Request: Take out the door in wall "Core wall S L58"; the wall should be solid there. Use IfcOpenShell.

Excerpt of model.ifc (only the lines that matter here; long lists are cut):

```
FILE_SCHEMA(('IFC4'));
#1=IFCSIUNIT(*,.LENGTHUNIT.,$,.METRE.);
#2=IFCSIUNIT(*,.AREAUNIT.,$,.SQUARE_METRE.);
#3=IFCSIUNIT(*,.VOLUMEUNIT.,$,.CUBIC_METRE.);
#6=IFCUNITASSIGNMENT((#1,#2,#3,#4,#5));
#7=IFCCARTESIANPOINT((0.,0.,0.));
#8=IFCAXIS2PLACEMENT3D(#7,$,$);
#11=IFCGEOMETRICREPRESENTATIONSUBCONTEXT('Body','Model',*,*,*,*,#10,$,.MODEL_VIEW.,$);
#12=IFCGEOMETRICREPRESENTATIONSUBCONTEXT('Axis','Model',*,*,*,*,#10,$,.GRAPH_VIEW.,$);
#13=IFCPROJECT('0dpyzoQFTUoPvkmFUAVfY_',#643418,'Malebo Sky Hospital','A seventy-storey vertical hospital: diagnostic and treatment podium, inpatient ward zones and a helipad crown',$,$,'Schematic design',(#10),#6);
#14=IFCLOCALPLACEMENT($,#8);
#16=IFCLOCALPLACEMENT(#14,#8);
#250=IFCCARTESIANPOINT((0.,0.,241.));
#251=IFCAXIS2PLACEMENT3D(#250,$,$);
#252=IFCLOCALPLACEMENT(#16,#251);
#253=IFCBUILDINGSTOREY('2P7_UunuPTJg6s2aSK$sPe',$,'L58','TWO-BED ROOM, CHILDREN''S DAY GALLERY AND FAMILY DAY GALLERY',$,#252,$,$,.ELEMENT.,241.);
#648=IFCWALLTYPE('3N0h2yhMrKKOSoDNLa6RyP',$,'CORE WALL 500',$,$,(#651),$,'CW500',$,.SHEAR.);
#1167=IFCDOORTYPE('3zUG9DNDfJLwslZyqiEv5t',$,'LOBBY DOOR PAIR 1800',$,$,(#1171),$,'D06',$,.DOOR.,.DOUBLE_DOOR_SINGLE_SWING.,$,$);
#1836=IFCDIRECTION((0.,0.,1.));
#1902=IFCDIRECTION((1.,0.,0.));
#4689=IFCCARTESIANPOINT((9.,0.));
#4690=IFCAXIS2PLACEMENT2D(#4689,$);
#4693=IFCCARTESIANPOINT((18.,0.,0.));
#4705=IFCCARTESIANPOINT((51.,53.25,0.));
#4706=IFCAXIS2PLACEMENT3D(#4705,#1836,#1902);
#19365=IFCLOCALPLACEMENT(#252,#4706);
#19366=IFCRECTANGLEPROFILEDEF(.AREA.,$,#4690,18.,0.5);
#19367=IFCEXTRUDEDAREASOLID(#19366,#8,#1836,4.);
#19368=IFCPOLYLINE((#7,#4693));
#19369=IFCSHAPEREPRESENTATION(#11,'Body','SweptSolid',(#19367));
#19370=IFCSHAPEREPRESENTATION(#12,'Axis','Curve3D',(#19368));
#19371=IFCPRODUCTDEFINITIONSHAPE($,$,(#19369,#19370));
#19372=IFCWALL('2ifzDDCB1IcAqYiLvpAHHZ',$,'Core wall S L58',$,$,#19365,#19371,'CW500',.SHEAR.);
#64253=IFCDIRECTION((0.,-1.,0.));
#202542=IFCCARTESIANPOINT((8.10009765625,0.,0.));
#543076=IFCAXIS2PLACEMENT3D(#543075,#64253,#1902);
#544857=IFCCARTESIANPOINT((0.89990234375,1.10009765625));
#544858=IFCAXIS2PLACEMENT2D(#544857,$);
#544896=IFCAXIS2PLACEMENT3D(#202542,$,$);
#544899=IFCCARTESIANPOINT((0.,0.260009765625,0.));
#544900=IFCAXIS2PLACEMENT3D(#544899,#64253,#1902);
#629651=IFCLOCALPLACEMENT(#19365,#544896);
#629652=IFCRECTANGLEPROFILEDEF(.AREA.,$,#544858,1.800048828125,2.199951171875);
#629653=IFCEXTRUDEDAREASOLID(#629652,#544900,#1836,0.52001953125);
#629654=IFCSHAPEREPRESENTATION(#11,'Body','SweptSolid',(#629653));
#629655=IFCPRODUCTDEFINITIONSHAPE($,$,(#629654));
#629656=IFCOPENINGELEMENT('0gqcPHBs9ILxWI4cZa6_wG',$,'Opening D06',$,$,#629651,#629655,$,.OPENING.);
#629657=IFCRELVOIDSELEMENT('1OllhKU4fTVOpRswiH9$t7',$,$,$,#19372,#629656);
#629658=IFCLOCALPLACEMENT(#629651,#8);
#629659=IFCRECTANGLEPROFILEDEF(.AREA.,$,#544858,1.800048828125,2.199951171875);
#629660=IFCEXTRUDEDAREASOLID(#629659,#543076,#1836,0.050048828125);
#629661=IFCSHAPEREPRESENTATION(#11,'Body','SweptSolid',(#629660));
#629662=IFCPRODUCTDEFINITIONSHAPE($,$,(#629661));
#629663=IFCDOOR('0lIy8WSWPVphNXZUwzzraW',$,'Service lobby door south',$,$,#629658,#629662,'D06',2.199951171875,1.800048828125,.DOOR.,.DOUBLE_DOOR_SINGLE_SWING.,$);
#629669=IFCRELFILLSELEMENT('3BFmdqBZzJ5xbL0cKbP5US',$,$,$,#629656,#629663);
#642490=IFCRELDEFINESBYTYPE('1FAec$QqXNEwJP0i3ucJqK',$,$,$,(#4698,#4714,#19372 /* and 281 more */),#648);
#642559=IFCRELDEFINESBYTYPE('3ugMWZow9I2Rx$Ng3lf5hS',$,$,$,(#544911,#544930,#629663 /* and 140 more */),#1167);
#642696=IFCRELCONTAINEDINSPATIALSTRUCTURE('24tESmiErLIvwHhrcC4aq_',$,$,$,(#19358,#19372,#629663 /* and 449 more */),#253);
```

```python
import ifcopenshell
import ifcopenshell.api.feature
import ifcopenshell.api.root
import ifcopenshell.geom
import ifcopenshell.util.shape

model = ifcopenshell.open("model.ifc")
settings = ifcopenshell.geom.settings()


def volume(element):
    """Net volume in cubic metres, openings subtracted."""
    shape = ifcopenshell.geom.create_shape(settings, element)
    return ifcopenshell.util.shape.get_volume(shape.geometry)


door = model.by_guid("0lIy8WSWPVphNXZUwzzraW")
opening = door.FillsVoids[0].RelatingOpeningElement
wall = opening.VoidsElements[0].RelatingBuildingElement
before = volume(wall)

ifcopenshell.api.root.remove_product(model, product=door)
ifcopenshell.api.feature.remove_feature(model, feature=opening)

after = volume(wall)

print(f"wall volume {before:.3f} -> {after:.3f} m3")

model.write("model_rev.ifc")
```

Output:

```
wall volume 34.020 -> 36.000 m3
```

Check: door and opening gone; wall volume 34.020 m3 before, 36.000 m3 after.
